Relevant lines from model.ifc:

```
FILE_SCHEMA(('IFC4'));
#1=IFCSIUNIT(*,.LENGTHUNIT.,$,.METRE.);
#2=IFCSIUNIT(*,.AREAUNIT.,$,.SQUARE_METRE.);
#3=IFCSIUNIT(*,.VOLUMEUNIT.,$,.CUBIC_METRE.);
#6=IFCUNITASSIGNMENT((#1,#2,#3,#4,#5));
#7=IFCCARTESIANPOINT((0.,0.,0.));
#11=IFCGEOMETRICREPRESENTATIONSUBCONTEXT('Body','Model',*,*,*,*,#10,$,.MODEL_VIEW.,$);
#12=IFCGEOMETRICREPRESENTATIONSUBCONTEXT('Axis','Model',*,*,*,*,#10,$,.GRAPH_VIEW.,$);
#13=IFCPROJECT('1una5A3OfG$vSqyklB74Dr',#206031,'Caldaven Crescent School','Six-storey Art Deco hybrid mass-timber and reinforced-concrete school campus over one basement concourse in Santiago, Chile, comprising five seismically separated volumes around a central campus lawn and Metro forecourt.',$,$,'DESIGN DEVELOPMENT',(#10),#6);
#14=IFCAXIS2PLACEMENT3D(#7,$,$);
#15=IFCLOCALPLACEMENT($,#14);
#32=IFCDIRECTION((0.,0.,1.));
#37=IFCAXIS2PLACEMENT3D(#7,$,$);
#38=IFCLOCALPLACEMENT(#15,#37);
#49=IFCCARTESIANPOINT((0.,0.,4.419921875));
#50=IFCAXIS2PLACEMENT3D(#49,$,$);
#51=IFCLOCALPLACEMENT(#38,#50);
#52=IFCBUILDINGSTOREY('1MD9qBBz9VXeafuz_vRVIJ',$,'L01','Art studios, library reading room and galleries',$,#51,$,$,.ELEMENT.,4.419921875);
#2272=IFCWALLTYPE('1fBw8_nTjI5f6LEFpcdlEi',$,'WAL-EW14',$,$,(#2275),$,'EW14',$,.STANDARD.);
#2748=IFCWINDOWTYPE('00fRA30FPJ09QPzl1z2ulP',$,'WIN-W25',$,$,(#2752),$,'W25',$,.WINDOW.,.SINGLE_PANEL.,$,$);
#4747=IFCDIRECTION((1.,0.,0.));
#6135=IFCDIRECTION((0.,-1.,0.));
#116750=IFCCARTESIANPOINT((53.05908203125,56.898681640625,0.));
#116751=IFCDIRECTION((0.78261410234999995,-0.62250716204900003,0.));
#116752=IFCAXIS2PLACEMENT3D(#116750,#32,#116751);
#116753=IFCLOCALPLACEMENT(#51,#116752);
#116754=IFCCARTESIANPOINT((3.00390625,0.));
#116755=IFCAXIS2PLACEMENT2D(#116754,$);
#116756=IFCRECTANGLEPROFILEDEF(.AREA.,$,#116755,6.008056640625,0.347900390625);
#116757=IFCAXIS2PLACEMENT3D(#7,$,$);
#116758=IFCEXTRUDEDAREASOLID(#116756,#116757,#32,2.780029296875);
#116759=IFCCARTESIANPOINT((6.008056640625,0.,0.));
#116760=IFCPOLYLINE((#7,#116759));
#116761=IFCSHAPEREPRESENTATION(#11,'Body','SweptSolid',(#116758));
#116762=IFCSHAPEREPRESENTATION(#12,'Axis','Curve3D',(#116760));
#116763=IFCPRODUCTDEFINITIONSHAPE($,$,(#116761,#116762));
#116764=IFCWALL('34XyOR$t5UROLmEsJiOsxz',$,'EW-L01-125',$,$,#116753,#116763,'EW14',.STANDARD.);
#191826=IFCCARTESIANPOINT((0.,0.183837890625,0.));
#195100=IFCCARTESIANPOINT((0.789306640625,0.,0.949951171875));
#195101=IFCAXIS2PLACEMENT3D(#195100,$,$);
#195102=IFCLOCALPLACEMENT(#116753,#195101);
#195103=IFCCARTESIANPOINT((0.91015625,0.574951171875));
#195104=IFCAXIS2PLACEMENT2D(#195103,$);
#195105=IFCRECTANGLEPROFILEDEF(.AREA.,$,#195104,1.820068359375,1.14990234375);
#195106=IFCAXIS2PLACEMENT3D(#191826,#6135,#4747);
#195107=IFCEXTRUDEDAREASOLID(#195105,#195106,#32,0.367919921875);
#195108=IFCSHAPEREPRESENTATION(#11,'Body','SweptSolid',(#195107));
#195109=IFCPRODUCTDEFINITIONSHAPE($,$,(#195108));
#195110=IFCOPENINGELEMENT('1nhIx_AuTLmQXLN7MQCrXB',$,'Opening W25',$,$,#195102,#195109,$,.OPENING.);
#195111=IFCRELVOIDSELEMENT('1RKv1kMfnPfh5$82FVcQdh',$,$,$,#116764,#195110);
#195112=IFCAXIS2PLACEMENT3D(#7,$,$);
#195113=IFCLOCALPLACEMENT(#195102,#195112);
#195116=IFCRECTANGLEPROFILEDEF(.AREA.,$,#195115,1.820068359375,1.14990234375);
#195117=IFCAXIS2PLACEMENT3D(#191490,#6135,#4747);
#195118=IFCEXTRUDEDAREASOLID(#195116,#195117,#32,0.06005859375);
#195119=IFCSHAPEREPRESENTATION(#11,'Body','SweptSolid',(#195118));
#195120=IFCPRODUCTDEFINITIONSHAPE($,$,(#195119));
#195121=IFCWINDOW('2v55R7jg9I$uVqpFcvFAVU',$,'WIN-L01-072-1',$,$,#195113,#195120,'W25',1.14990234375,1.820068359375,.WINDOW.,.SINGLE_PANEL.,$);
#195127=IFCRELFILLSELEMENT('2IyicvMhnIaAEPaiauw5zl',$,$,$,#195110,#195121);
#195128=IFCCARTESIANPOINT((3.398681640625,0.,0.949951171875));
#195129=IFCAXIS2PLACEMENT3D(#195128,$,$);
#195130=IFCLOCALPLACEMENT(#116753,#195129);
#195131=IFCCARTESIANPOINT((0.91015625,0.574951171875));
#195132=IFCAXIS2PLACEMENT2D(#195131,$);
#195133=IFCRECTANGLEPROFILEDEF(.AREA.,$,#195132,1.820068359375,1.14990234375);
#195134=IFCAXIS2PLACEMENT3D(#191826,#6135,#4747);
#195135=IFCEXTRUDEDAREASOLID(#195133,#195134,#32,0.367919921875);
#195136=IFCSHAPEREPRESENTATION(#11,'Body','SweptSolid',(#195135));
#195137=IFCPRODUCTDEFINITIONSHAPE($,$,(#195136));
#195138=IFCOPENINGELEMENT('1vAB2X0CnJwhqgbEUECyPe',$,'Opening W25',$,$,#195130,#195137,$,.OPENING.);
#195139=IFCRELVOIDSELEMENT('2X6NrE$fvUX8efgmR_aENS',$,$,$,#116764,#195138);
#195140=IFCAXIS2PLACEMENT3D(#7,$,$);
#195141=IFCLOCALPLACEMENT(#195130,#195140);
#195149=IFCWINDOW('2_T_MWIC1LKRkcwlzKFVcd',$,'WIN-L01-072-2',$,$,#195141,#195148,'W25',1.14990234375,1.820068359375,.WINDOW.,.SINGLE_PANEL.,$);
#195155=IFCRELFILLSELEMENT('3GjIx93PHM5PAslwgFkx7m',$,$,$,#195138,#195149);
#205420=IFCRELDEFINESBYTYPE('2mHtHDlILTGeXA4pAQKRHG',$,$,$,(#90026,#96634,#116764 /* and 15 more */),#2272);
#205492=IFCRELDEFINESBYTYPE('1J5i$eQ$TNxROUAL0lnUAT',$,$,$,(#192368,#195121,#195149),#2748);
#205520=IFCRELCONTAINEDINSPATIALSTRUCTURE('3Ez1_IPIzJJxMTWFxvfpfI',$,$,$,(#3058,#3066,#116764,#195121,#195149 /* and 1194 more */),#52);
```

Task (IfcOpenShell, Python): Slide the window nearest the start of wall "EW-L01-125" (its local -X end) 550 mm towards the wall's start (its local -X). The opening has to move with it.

```python
import ifcopenshell
import ifcopenshell.api.geometry
import ifcopenshell.util.placement

model = ifcopenshell.open("model.ifc")

window = model.by_id(195121)
opening = window.FillsVoids[0].RelatingOpeningElement
wall = opening.VoidsElements[0].RelatingBuildingElement

wall_matrix = ifcopenshell.util.placement.get_local_placement(wall.ObjectPlacement)
shift = wall_matrix[:3, 0] * -0.55
before = ifcopenshell.util.placement.get_local_placement(window.ObjectPlacement)[:3, 3].copy()

# The window is placed relative to its opening, so it follows when the opening moves.
matrix = ifcopenshell.util.placement.get_local_placement(opening.ObjectPlacement)
matrix[:3, 3] += shift
ifcopenshell.api.geometry.edit_object_placement(
    model, product=opening, matrix=matrix, is_si=False, should_transform_children=True
)

after = ifcopenshell.util.placement.get_local_placement(window.ObjectPlacement)[:3, 3]
print("window moved by", (after - before).round(3) + 0.0)

model.write("model-out.ifc")
```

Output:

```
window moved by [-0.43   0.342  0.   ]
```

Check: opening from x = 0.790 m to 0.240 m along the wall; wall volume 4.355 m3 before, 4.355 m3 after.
